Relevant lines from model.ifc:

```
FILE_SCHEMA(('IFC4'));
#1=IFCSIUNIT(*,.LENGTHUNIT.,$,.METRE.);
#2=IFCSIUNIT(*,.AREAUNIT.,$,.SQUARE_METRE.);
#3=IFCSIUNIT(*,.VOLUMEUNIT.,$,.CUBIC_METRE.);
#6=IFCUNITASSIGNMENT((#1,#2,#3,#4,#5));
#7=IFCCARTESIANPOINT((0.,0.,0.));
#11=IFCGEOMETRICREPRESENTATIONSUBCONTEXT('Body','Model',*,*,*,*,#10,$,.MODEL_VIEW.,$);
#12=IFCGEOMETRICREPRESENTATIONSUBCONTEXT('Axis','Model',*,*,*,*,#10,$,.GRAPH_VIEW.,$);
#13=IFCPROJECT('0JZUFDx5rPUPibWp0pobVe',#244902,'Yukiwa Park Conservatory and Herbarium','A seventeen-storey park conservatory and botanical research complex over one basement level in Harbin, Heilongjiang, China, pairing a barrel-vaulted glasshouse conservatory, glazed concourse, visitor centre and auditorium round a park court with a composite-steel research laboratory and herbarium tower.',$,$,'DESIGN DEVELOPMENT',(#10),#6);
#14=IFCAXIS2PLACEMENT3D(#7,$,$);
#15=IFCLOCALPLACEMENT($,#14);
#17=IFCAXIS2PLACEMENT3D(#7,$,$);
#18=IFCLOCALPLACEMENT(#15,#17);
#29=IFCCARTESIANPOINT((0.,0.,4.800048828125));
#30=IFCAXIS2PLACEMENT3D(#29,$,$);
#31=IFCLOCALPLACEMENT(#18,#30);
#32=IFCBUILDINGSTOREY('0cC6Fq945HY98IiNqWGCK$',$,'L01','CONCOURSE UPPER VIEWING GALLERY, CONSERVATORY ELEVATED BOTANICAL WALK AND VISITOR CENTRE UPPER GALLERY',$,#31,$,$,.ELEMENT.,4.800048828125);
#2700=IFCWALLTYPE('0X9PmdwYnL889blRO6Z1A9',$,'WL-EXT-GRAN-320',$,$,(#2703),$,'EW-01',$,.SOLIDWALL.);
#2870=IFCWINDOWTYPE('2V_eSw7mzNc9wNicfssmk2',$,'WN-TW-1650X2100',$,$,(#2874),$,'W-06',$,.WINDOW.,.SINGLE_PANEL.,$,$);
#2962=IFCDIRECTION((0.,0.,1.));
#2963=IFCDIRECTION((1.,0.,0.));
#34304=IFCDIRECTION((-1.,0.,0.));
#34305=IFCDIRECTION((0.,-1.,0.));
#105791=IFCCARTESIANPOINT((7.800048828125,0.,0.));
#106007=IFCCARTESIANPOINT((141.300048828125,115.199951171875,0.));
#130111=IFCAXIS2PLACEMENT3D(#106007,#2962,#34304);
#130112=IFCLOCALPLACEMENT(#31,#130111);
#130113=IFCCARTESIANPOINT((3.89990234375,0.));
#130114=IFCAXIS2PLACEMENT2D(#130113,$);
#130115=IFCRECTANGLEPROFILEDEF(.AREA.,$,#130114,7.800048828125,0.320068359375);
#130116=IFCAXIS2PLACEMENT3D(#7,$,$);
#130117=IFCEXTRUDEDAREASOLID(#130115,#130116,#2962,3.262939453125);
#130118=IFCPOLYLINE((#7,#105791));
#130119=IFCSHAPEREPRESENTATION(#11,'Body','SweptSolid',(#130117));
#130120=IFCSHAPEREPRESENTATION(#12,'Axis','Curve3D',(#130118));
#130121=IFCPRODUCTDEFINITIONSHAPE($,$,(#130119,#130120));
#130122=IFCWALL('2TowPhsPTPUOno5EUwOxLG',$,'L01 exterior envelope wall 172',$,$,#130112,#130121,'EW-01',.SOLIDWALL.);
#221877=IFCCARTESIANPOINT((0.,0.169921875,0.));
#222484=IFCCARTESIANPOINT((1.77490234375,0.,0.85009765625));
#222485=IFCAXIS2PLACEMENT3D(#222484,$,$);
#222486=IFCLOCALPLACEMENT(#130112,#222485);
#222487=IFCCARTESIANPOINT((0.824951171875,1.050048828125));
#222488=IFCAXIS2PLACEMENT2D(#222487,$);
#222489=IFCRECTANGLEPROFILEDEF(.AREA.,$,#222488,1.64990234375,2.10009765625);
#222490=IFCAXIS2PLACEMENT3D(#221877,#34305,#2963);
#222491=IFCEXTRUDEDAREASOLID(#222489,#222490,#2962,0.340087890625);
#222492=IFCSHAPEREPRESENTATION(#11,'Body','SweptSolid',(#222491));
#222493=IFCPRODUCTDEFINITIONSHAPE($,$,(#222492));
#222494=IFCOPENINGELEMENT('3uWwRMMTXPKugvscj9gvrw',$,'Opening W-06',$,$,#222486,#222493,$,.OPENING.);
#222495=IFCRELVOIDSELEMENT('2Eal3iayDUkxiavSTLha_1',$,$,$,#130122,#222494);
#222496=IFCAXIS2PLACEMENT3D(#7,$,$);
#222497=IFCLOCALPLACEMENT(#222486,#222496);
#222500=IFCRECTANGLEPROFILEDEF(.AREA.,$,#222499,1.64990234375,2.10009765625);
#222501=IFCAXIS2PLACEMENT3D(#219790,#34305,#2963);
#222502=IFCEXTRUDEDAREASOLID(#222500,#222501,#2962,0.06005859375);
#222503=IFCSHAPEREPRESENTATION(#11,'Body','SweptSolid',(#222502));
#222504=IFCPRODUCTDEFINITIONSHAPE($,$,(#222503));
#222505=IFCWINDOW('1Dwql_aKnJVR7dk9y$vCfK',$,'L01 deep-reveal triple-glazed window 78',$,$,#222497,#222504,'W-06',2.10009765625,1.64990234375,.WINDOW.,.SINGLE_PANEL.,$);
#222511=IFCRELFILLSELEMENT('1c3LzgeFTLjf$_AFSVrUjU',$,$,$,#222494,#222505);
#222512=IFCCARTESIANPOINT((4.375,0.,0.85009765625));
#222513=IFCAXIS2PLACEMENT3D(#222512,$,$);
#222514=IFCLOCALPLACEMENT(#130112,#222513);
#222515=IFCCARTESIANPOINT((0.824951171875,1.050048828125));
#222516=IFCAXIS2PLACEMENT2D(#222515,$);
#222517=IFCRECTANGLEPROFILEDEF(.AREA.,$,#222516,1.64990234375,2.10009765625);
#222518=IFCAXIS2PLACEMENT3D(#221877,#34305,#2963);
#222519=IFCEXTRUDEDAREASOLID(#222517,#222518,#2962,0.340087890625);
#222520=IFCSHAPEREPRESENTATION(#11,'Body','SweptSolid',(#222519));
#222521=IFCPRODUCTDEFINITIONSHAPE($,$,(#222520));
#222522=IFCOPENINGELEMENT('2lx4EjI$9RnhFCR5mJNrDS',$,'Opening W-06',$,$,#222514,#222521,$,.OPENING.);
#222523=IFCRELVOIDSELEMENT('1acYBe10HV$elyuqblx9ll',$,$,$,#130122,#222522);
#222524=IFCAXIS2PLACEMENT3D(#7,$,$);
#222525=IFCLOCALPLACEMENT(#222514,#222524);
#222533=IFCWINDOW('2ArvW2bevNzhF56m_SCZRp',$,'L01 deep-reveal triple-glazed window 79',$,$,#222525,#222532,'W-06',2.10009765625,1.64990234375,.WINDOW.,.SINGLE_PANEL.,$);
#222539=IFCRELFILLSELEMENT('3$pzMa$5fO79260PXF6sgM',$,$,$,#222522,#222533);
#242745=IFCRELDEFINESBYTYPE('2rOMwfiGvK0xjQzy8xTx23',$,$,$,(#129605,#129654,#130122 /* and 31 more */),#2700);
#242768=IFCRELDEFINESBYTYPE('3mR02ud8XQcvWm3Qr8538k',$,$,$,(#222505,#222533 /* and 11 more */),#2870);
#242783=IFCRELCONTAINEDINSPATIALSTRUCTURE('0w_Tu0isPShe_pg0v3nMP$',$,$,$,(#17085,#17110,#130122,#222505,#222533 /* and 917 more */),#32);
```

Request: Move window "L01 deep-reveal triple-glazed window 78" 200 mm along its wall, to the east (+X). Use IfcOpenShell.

```python
import ifcopenshell
import ifcopenshell.api.geometry
import ifcopenshell.util.placement
import ifcopenshell.util.unit

model = ifcopenshell.open("model.ifc")
unit_scale = ifcopenshell.util.unit.calculate_unit_scale(model)

window = model.by_id(222505)
opening = window.FillsVoids[0].RelatingOpeningElement
wall = opening.VoidsElements[0].RelatingBuildingElement

wall_matrix = ifcopenshell.util.placement.get_local_placement(wall.ObjectPlacement)
shift = wall_matrix[:3, 0] * -0.2 / unit_scale
before = ifcopenshell.util.placement.get_local_placement(window.ObjectPlacement)[:3, 3].copy()

# The window is placed relative to its opening, so it follows when the opening moves.
matrix = ifcopenshell.util.placement.get_local_placement(opening.ObjectPlacement)
matrix[:3, 3] += shift
ifcopenshell.api.geometry.edit_object_placement(
    model, product=opening, matrix=matrix, is_si=False, should_transform_children=True
)

after = ifcopenshell.util.placement.get_local_placement(window.ObjectPlacement)[:3, 3]
print("window moved by", (after - before).round(3) + 0.0)

model.write("model-out.ifc")
```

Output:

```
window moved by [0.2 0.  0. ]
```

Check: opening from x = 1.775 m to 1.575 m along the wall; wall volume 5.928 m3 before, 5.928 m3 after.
